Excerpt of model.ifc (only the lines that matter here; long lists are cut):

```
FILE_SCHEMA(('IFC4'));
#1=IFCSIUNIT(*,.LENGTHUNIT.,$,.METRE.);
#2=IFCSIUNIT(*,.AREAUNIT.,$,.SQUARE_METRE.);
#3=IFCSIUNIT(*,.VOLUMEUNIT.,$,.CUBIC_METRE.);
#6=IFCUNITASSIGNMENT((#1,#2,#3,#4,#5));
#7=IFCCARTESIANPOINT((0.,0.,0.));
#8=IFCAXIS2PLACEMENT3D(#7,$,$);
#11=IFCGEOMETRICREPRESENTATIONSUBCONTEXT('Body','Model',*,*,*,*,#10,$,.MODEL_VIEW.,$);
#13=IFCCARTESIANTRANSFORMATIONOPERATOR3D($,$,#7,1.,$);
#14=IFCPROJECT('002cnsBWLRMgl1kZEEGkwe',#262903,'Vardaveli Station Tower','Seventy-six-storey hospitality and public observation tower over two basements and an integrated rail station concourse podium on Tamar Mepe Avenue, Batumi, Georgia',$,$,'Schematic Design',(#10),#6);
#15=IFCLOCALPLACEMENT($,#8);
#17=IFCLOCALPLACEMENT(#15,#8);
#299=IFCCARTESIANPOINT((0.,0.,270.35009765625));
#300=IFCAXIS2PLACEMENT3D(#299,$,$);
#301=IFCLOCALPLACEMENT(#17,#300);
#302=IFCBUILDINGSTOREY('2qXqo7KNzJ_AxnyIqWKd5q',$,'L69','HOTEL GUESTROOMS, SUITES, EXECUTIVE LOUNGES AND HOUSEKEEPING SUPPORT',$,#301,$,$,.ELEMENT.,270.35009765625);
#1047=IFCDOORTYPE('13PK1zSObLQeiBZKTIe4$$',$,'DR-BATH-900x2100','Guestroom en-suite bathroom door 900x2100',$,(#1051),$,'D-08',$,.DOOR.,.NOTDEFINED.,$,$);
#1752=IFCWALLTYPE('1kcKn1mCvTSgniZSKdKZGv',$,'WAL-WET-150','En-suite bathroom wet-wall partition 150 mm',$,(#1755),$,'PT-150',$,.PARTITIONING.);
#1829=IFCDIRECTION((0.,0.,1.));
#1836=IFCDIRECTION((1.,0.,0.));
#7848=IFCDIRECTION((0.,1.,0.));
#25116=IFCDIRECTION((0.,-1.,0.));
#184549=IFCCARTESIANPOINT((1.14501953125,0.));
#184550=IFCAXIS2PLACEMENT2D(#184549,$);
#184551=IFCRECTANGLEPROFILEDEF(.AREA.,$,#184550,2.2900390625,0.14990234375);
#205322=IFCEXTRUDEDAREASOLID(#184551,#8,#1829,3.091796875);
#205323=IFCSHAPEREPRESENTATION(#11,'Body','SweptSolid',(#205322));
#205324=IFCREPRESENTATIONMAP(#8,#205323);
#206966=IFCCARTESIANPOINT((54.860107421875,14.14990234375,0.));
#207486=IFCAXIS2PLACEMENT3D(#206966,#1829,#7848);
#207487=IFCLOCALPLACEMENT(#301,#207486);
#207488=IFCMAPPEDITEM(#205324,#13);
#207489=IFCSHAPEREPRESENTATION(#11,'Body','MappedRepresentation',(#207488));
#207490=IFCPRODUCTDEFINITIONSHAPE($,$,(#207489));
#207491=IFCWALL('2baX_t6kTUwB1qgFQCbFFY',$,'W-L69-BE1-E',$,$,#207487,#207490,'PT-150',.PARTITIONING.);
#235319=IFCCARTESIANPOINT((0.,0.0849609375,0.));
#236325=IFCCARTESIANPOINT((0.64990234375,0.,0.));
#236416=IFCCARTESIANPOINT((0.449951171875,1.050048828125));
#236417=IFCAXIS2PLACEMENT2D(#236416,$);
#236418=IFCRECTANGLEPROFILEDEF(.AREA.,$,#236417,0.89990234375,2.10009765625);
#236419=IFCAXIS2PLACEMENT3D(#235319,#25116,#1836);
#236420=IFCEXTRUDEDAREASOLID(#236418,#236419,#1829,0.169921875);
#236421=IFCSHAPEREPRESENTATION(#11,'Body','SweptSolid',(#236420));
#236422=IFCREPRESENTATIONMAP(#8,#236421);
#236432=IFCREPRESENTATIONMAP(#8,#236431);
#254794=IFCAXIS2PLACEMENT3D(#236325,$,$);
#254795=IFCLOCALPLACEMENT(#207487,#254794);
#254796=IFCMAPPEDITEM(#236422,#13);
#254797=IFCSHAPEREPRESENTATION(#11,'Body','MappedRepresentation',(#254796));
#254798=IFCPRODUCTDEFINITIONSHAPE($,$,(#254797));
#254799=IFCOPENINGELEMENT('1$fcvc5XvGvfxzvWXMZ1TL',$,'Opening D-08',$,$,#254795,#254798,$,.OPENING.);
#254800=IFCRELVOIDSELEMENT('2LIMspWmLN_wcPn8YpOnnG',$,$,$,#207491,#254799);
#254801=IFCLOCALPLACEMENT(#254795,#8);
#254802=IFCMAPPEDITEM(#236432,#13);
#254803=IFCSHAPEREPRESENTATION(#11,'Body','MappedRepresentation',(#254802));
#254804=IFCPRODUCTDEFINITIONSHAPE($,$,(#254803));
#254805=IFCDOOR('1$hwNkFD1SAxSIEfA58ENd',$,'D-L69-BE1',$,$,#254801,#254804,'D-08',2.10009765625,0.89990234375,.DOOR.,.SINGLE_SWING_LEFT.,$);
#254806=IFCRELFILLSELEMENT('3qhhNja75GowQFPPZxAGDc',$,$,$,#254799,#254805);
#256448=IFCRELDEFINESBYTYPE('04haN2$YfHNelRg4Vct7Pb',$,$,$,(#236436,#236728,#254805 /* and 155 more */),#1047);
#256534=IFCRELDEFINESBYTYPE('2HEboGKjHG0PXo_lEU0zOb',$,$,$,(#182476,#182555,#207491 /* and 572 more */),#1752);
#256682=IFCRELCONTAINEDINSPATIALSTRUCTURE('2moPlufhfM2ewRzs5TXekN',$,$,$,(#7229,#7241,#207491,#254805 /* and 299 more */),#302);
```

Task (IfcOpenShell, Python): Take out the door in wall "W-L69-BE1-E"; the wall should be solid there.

```python
import ifcopenshell
import ifcopenshell.api.feature
import ifcopenshell.api.root
import ifcopenshell.geom
import ifcopenshell.util.shape

model = ifcopenshell.open("model.ifc")
settings = ifcopenshell.geom.settings()


def volume(element):
    """Net volume in cubic metres, openings subtracted."""
    shape = ifcopenshell.geom.create_shape(settings, element)
    return ifcopenshell.util.shape.get_volume(shape.geometry)


door = model.by_guid("1$hwNkFD1SAxSIEfA58ENd")
opening = door.FillsVoids[0].RelatingOpeningElement
wall = opening.VoidsElements[0].RelatingBuildingElement
before = volume(wall)

ifcopenshell.api.root.remove_product(model, product=door)
ifcopenshell.api.feature.remove_feature(model, feature=opening)

after = volume(wall)

print(f"wall volume {before:.3f} -> {after:.3f} m3")

model.write("model_rev.ifc")
```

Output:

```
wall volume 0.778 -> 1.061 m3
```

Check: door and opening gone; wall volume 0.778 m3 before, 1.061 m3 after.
